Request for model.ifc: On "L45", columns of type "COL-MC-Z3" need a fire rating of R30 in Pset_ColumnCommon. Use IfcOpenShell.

First a look at what the model holds.

```python
import ifcopenshell
import ifcopenshell.util.element

model = ifcopenshell.open("model.ifc")
print(model.schema)
storey = next(s for s in model.by_type("IfcBuildingStorey") if s.Name == "L45")
columns = [e for e in ifcopenshell.util.element.get_decomposition(storey) if e.is_a("IfcColumn")]
seen = {}
for e in columns:
    element_type = ifcopenshell.util.element.get_type(e)
    key = (element_type.Name if element_type != e and element_type else None, ifcopenshell.util.element.get_pset(e, "Pset_ColumnCommon", "FireRating"))
    seen[key] = seen.get(key, 0) + 1
for (name, value), count in sorted(seen.items(), key=str):
    print(count, "x", name, "|", value)
```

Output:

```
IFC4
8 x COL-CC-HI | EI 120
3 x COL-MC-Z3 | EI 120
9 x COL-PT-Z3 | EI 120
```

```python
import ifcopenshell
import ifcopenshell.api.pset
import ifcopenshell.util.element

model = ifcopenshell.open("model.ifc")

storey = next(s for s in model.by_type("IfcBuildingStorey") if s.Name == "L45")
columns = [e for e in ifcopenshell.util.element.get_decomposition(storey) if e.is_a("IfcColumn")]

count = 0
for e in columns:
    element_type = ifcopenshell.util.element.get_type(e)
    if element_type in (None, e) or element_type.Name != "COL-MC-Z3":
        continue
    found = ifcopenshell.util.element.get_pset(e, "Pset_ColumnCommon", should_inherit=False)
    if found:
        pset = model.by_id(found["id"])
        if len(ifcopenshell.util.element.get_elements_by_pset(pset)) > 1:
            pset = ifcopenshell.api.pset.unshare_pset(model, products=[e], pset=pset)[0]
    else:
        pset = ifcopenshell.api.pset.add_pset(model, product=e, name="Pset_ColumnCommon")
    ifcopenshell.api.pset.edit_pset(model, pset=pset, properties={"FireRating": "R30"})
    count += 1

print(count, "columns updated")

model.write("model_rev.ifc")
```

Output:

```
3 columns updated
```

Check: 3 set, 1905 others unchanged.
